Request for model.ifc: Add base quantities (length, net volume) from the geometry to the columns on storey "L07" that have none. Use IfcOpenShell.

First a look at what the model holds.

```python
import ifcopenshell
import ifcopenshell.util.element
import ifcopenshell.util.unit

model = ifcopenshell.open("model.ifc")
print(model.schema)
for unit_type in ("LENGTHUNIT", "AREAUNIT", "VOLUMEUNIT"):
    print(unit_type, ifcopenshell.util.unit.calculate_unit_scale(model, unit_type))
storey = next(s for s in model.by_type("IfcBuildingStorey") if s.Name == "L07")
columns = [e for e in ifcopenshell.util.element.get_decomposition(storey) if e.is_a("IfcColumn")]
for e in sorted(columns, key=lambda e: e.id()):
    print(e.id(), e.is_a(), e.Name, list(ifcopenshell.util.element.get_psets(e, qtos_only=True)), sep=" | ")
```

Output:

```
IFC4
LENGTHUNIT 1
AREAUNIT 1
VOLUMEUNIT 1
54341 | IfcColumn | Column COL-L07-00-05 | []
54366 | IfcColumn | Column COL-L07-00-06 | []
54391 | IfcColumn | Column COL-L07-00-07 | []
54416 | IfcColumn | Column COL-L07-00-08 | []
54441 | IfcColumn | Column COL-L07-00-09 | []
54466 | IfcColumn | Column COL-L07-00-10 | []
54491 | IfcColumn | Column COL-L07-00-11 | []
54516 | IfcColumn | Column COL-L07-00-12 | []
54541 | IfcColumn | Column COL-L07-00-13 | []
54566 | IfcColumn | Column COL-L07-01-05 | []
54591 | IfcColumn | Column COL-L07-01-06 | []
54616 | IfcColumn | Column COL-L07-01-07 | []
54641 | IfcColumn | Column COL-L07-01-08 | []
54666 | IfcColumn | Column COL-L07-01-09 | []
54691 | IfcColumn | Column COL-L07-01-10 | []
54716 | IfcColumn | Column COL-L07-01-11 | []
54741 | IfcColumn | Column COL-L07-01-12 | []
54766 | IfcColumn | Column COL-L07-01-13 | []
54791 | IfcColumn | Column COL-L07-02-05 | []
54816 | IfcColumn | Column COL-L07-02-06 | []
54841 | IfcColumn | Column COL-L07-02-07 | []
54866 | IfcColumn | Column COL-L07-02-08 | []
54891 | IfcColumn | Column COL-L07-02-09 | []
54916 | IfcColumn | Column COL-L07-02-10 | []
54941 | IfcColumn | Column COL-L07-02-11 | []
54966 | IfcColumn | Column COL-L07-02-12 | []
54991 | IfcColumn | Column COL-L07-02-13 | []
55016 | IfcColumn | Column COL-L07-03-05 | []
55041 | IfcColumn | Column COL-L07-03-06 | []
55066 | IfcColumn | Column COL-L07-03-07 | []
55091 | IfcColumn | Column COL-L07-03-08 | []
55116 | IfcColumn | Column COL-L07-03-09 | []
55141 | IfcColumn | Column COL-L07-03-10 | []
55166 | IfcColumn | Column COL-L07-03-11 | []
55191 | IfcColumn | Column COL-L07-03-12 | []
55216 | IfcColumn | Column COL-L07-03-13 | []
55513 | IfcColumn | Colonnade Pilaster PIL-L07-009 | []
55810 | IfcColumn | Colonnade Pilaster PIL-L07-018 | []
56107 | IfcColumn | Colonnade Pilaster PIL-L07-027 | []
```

```python
import ifcopenshell
import ifcopenshell.api.pset
import ifcopenshell.geom
import ifcopenshell.util.element
import ifcopenshell.util.shape
import ifcopenshell.util.unit

model = ifcopenshell.open("model.ifc")
unit_scale = ifcopenshell.util.unit.calculate_unit_scale(model)
volume_scale = ifcopenshell.util.unit.calculate_unit_scale(model, "VOLUMEUNIT")
settings = ifcopenshell.geom.settings()

storey = next(s for s in model.by_type("IfcBuildingStorey") if s.Name == "L07")
columns = [e for e in ifcopenshell.util.element.get_decomposition(storey) if e.is_a("IfcColumn")]

for e in sorted(columns, key=lambda e: e.id()):
    if ifcopenshell.util.element.get_psets(e, qtos_only=True, should_inherit=False):
        continue
    # Geometry comes back in metres, in the element's own axes.
    shape = ifcopenshell.geom.create_shape(settings, e)
    values = {
        "Length": ifcopenshell.util.shape.get_z(shape.geometry) / unit_scale,
        "NetVolume": ifcopenshell.util.shape.get_volume(shape.geometry) / volume_scale,
    }
    qto = ifcopenshell.api.pset.add_qto(model, product=e, name="Qto_ColumnBaseQuantities")
    ifcopenshell.api.pset.edit_qto(model, qto=qto, properties=values)
    print(e.id(), {k: round(v, 3) for k, v in values.items()})

model.write("model_rev.ifc")
```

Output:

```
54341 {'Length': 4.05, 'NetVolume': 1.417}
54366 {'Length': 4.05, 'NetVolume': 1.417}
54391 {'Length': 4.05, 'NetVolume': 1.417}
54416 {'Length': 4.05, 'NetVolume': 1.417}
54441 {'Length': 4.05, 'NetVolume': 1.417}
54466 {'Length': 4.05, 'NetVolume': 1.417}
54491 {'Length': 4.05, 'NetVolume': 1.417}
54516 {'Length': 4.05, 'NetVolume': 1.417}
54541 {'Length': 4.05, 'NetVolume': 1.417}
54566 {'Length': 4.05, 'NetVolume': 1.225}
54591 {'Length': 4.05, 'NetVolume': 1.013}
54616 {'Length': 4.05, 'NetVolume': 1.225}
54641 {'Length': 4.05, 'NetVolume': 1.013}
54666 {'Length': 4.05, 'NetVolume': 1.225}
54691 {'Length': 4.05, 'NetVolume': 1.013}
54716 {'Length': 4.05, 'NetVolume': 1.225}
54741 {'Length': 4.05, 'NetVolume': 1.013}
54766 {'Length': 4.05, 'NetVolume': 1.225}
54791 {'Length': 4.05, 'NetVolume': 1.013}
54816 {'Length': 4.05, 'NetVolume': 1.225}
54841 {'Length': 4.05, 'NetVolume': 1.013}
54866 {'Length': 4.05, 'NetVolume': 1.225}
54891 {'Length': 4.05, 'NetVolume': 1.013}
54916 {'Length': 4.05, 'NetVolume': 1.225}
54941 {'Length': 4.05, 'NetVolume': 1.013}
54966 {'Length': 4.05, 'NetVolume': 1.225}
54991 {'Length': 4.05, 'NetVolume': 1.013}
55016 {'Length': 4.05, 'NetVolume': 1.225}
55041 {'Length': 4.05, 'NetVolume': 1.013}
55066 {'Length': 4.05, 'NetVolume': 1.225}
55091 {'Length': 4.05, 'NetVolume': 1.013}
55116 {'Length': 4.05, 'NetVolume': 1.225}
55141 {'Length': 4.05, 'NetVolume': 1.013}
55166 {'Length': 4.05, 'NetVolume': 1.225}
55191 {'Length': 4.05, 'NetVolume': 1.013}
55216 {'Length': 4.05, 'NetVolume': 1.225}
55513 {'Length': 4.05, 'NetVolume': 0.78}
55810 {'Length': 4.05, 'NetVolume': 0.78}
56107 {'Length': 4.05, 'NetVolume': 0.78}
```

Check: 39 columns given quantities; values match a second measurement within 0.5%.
